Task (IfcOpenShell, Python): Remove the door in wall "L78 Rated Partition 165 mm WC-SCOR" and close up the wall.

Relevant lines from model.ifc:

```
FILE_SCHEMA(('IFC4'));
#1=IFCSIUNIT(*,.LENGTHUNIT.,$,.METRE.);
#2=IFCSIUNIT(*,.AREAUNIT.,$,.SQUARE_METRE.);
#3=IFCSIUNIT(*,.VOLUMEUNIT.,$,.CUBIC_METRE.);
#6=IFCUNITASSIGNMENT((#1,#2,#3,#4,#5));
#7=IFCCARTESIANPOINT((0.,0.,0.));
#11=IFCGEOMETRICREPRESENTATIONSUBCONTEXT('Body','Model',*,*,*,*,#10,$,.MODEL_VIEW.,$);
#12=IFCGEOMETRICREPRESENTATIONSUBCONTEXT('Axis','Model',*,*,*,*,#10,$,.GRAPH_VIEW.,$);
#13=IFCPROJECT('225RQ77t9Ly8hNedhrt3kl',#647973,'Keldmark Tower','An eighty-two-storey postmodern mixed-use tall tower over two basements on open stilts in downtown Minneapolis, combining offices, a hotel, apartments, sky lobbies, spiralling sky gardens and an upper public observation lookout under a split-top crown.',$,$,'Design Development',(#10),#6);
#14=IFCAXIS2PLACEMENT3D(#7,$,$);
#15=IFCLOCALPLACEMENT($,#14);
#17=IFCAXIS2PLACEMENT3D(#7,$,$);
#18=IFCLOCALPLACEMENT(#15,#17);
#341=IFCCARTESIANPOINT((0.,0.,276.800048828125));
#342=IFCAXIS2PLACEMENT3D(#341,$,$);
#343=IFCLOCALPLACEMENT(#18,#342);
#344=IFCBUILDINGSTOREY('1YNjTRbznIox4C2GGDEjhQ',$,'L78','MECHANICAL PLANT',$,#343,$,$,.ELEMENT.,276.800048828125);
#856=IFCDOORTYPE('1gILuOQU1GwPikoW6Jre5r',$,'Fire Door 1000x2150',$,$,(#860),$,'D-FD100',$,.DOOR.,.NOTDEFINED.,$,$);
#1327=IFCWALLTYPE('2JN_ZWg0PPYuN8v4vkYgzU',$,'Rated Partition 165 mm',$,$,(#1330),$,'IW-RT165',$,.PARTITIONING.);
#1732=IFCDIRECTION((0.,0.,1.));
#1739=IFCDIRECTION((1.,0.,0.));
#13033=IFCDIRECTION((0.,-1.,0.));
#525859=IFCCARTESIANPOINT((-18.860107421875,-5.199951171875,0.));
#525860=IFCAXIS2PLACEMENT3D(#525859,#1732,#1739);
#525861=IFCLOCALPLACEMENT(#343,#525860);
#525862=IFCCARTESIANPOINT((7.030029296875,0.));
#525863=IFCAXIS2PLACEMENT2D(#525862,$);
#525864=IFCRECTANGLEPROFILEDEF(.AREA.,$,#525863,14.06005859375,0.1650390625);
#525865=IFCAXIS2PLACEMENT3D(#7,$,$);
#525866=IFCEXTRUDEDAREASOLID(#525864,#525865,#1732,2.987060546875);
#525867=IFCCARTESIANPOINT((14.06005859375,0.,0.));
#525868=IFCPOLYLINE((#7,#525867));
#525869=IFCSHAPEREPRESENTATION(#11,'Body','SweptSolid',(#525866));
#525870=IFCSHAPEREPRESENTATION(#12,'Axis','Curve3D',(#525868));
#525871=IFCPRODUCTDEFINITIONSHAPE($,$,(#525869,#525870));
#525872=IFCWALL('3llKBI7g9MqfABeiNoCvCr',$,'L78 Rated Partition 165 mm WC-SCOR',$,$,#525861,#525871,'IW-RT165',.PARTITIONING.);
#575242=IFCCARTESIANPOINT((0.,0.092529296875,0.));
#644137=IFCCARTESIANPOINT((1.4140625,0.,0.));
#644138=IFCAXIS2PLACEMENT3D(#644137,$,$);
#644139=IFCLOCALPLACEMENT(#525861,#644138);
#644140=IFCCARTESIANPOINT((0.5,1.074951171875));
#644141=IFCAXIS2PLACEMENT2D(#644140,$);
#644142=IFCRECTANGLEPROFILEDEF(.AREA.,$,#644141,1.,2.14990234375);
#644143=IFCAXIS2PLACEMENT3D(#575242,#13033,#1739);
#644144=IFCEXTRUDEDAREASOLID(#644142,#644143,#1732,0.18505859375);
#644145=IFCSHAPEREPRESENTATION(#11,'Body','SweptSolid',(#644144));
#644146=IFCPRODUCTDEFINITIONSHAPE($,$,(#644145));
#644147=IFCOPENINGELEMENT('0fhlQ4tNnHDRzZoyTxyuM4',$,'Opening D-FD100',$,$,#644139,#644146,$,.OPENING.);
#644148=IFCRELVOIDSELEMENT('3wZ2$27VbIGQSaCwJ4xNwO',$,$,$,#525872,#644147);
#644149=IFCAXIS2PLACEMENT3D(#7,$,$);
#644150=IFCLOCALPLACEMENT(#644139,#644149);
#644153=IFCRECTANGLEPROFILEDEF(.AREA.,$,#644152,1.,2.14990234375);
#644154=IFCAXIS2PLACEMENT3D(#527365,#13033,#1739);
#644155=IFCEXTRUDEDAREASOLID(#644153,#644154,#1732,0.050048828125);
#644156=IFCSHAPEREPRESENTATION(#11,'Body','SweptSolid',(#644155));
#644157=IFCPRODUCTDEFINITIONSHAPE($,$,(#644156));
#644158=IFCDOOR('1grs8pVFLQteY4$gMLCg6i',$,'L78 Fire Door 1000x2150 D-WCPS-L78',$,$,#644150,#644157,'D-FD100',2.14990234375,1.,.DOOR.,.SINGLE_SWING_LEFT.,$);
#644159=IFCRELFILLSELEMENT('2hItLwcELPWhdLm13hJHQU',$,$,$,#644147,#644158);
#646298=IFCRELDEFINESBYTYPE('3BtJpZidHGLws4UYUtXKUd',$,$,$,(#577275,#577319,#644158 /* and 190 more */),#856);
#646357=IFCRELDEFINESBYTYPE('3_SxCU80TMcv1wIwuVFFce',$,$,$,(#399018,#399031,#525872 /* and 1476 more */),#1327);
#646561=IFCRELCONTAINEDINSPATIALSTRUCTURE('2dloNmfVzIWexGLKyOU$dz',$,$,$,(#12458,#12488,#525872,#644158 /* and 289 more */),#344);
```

```python
import ifcopenshell
import ifcopenshell.api.feature
import ifcopenshell.api.root
import ifcopenshell.geom
import ifcopenshell.util.shape

model = ifcopenshell.open("model.ifc")
settings = ifcopenshell.geom.settings()


def volume(element):
    """Net volume in cubic metres, openings subtracted."""
    shape = ifcopenshell.geom.create_shape(settings, element)
    return ifcopenshell.util.shape.get_volume(shape.geometry)


door = model.by_guid("1grs8pVFLQteY4$gMLCg6i")
opening = door.FillsVoids[0].RelatingOpeningElement
wall = opening.VoidsElements[0].RelatingBuildingElement
before = volume(wall)

ifcopenshell.api.root.remove_product(model, product=door)
ifcopenshell.api.feature.remove_feature(model, feature=opening)

after = volume(wall)

print(f"wall volume {before:.3f} -> {after:.3f} m3")

model.write("model_v2.ifc")
```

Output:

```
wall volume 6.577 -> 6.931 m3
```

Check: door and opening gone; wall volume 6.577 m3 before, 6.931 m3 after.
